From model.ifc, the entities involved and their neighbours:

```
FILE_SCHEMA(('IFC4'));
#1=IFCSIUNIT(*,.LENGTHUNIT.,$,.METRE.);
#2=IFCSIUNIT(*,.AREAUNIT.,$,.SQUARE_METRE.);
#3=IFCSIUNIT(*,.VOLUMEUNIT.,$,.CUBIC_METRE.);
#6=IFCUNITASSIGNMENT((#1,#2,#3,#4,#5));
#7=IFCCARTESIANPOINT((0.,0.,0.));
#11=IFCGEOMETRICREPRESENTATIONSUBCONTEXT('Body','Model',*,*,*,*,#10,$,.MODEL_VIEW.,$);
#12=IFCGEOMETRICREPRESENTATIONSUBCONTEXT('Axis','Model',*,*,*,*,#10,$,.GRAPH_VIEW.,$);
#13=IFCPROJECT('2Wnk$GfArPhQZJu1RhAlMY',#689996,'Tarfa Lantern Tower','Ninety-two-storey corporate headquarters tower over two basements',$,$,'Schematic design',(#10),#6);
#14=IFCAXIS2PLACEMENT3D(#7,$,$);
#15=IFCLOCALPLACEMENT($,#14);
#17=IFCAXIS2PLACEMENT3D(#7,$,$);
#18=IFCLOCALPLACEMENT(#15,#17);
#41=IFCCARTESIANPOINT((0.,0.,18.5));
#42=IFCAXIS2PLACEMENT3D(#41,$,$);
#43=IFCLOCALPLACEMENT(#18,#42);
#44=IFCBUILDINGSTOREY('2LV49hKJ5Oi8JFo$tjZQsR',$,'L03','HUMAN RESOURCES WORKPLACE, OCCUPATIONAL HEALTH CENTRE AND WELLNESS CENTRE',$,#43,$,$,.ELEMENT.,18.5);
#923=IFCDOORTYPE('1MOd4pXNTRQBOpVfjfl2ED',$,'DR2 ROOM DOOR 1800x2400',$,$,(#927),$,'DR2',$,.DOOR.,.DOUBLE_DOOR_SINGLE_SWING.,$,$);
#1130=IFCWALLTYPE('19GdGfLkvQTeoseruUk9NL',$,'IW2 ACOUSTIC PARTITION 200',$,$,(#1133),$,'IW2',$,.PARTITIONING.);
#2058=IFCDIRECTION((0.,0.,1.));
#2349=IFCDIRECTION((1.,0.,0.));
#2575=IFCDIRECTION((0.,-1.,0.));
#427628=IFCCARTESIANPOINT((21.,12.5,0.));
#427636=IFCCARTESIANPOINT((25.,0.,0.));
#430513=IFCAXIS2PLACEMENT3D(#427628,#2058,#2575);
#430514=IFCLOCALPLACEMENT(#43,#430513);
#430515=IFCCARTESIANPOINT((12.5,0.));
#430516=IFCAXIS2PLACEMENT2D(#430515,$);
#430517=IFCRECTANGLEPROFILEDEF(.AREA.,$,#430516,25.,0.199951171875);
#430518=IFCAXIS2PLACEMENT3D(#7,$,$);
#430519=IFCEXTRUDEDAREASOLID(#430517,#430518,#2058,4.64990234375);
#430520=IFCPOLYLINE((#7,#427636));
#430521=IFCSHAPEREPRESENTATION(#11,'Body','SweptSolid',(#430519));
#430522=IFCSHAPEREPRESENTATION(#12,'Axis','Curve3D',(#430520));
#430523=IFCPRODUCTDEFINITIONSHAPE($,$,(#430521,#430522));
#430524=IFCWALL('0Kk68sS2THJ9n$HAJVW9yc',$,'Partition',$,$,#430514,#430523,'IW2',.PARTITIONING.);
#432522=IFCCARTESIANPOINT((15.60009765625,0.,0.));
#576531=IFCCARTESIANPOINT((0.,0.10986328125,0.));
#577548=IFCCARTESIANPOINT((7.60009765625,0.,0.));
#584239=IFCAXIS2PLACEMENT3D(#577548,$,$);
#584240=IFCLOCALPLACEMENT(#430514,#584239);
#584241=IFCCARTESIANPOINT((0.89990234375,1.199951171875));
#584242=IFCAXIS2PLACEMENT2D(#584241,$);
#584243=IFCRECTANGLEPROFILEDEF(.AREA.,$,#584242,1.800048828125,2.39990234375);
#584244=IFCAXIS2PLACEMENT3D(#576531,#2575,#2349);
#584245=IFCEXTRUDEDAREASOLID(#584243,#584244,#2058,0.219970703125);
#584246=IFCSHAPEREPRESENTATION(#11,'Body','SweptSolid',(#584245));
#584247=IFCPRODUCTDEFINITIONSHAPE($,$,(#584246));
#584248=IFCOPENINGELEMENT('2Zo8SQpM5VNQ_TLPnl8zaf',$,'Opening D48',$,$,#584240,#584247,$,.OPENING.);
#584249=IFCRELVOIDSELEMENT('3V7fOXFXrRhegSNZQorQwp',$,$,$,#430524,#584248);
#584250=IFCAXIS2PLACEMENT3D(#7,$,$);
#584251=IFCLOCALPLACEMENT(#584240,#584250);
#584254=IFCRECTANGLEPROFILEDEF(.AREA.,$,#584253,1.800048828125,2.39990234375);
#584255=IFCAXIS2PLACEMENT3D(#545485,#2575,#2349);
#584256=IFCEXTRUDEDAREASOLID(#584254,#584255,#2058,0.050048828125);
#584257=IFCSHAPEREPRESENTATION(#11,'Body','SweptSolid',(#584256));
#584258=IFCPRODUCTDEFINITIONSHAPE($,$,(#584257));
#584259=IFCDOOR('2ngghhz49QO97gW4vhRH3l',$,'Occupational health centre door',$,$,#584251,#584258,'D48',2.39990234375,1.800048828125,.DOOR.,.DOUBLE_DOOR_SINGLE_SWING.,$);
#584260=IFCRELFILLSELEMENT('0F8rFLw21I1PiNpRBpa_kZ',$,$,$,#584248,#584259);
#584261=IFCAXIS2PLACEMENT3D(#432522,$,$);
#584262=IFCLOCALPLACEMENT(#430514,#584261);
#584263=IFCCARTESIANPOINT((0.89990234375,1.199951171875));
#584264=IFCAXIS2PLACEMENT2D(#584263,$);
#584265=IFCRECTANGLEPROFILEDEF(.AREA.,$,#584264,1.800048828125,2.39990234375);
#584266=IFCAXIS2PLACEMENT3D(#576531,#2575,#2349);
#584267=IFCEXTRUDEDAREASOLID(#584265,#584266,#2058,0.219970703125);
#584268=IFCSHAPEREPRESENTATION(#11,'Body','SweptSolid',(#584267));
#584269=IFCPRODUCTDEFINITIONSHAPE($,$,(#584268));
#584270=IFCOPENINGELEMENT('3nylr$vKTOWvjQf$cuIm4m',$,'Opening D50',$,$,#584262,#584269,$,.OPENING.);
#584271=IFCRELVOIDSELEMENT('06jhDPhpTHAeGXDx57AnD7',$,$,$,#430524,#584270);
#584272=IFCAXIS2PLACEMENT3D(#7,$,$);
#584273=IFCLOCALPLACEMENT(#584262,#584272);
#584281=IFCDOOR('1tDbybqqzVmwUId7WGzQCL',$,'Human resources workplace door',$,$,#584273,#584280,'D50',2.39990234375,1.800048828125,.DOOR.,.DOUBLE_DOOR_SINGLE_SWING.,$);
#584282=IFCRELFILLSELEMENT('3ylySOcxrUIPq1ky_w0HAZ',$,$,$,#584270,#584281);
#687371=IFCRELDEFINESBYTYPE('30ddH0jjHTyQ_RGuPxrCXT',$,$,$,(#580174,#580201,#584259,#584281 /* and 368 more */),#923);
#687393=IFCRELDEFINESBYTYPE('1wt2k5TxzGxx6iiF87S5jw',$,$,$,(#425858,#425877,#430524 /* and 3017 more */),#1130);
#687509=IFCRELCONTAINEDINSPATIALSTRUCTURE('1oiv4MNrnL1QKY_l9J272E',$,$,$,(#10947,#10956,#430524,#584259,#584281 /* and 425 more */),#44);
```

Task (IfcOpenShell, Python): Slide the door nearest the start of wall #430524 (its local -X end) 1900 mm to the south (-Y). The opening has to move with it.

```python
import ifcopenshell
import ifcopenshell.api.geometry
import ifcopenshell.util.placement

model = ifcopenshell.open("model.ifc")

door = model.by_guid("2ngghhz49QO97gW4vhRH3l")
opening = door.FillsVoids[0].RelatingOpeningElement
wall = opening.VoidsElements[0].RelatingBuildingElement

wall_matrix = ifcopenshell.util.placement.get_local_placement(wall.ObjectPlacement)
shift = wall_matrix[:3, 0] * 1.9
before = ifcopenshell.util.placement.get_local_placement(door.ObjectPlacement)[:3, 3].copy()

# The door is placed relative to its opening, so it follows when the opening moves.
matrix = ifcopenshell.util.placement.get_local_placement(opening.ObjectPlacement)
matrix[:3, 3] += shift
ifcopenshell.api.geometry.edit_object_placement(
    model, product=opening, matrix=matrix, is_si=False, should_transform_children=True
)

after = ifcopenshell.util.placement.get_local_placement(door.ObjectPlacement)[:3, 3]
print("door moved by", (after - before).round(3) + 0.0)

model.write("model_v2.ifc")
```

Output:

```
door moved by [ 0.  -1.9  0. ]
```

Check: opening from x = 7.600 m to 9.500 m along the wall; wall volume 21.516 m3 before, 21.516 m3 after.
